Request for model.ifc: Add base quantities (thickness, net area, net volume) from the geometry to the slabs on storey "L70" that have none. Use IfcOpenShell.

First a look at what the model holds.

```python
import ifcopenshell
import ifcopenshell.util.element
import ifcopenshell.util.unit

model = ifcopenshell.open("model.ifc")
print(model.schema)
for unit_type in ("LENGTHUNIT", "AREAUNIT", "VOLUMEUNIT"):
    print(unit_type, ifcopenshell.util.unit.calculate_unit_scale(model, unit_type))
storey = next(s for s in model.by_type("IfcBuildingStorey") if s.Name == "L70")
slabs = [e for e in ifcopenshell.util.element.get_decomposition(storey) if e.is_a("IfcSlab")]
for e in sorted(slabs, key=lambda e: e.id()):
    print(e.id(), e.is_a(), e.Name, list(ifcopenshell.util.element.get_psets(e, qtos_only=True)), sep=" | ")
```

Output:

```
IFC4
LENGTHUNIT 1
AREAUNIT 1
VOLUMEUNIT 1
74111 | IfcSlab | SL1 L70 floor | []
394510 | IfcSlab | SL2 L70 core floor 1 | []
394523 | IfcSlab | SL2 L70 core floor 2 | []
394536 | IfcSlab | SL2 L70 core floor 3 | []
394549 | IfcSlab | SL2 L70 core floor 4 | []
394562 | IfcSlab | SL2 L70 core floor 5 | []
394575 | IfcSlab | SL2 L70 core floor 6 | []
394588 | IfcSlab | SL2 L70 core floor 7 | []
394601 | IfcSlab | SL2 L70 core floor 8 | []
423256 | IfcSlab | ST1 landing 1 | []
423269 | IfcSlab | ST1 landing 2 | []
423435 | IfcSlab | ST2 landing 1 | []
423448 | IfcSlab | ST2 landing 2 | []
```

```python
import ifcopenshell
import ifcopenshell.api.pset
import ifcopenshell.geom
import ifcopenshell.util.element
import ifcopenshell.util.shape
import ifcopenshell.util.unit

model = ifcopenshell.open("model.ifc")
unit_scale = ifcopenshell.util.unit.calculate_unit_scale(model)
area_scale = ifcopenshell.util.unit.calculate_unit_scale(model, "AREAUNIT")
volume_scale = ifcopenshell.util.unit.calculate_unit_scale(model, "VOLUMEUNIT")
settings = ifcopenshell.geom.settings()

storey = next(s for s in model.by_type("IfcBuildingStorey") if s.Name == "L70")
slabs = [e for e in ifcopenshell.util.element.get_decomposition(storey) if e.is_a("IfcSlab")]

for e in sorted(slabs, key=lambda e: e.id()):
    if ifcopenshell.util.element.get_psets(e, qtos_only=True, should_inherit=False):
        continue
    # Geometry comes back in metres, in the element's own axes.
    shape = ifcopenshell.geom.create_shape(settings, e)
    values = {
        "Width": ifcopenshell.util.shape.get_z(shape.geometry) / unit_scale,
        "NetArea": ifcopenshell.util.shape.get_footprint_area(shape.geometry) / area_scale,
        "NetVolume": ifcopenshell.util.shape.get_volume(shape.geometry) / volume_scale,
    }
    qto = ifcopenshell.api.pset.add_qto(model, product=e, name="Qto_SlabBaseQuantities")
    ifcopenshell.api.pset.edit_qto(model, qto=qto, properties=values)
    print(e.id(), {k: round(v, 3) for k, v in values.items()})

model.write("model_updated.ifc")
```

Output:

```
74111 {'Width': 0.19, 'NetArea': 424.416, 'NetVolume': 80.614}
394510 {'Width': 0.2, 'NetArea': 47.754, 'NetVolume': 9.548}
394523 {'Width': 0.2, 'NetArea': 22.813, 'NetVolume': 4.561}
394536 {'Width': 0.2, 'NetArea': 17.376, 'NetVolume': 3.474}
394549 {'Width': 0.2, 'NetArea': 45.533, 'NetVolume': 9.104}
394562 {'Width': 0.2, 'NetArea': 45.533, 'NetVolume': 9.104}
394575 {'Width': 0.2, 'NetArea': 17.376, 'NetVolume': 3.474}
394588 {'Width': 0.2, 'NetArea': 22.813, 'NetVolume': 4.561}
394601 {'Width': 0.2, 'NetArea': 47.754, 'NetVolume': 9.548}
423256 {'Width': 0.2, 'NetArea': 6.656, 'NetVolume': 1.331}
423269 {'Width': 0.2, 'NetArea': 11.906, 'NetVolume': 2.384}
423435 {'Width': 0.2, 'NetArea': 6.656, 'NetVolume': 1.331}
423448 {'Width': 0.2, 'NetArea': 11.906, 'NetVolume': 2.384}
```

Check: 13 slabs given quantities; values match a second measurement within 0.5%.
